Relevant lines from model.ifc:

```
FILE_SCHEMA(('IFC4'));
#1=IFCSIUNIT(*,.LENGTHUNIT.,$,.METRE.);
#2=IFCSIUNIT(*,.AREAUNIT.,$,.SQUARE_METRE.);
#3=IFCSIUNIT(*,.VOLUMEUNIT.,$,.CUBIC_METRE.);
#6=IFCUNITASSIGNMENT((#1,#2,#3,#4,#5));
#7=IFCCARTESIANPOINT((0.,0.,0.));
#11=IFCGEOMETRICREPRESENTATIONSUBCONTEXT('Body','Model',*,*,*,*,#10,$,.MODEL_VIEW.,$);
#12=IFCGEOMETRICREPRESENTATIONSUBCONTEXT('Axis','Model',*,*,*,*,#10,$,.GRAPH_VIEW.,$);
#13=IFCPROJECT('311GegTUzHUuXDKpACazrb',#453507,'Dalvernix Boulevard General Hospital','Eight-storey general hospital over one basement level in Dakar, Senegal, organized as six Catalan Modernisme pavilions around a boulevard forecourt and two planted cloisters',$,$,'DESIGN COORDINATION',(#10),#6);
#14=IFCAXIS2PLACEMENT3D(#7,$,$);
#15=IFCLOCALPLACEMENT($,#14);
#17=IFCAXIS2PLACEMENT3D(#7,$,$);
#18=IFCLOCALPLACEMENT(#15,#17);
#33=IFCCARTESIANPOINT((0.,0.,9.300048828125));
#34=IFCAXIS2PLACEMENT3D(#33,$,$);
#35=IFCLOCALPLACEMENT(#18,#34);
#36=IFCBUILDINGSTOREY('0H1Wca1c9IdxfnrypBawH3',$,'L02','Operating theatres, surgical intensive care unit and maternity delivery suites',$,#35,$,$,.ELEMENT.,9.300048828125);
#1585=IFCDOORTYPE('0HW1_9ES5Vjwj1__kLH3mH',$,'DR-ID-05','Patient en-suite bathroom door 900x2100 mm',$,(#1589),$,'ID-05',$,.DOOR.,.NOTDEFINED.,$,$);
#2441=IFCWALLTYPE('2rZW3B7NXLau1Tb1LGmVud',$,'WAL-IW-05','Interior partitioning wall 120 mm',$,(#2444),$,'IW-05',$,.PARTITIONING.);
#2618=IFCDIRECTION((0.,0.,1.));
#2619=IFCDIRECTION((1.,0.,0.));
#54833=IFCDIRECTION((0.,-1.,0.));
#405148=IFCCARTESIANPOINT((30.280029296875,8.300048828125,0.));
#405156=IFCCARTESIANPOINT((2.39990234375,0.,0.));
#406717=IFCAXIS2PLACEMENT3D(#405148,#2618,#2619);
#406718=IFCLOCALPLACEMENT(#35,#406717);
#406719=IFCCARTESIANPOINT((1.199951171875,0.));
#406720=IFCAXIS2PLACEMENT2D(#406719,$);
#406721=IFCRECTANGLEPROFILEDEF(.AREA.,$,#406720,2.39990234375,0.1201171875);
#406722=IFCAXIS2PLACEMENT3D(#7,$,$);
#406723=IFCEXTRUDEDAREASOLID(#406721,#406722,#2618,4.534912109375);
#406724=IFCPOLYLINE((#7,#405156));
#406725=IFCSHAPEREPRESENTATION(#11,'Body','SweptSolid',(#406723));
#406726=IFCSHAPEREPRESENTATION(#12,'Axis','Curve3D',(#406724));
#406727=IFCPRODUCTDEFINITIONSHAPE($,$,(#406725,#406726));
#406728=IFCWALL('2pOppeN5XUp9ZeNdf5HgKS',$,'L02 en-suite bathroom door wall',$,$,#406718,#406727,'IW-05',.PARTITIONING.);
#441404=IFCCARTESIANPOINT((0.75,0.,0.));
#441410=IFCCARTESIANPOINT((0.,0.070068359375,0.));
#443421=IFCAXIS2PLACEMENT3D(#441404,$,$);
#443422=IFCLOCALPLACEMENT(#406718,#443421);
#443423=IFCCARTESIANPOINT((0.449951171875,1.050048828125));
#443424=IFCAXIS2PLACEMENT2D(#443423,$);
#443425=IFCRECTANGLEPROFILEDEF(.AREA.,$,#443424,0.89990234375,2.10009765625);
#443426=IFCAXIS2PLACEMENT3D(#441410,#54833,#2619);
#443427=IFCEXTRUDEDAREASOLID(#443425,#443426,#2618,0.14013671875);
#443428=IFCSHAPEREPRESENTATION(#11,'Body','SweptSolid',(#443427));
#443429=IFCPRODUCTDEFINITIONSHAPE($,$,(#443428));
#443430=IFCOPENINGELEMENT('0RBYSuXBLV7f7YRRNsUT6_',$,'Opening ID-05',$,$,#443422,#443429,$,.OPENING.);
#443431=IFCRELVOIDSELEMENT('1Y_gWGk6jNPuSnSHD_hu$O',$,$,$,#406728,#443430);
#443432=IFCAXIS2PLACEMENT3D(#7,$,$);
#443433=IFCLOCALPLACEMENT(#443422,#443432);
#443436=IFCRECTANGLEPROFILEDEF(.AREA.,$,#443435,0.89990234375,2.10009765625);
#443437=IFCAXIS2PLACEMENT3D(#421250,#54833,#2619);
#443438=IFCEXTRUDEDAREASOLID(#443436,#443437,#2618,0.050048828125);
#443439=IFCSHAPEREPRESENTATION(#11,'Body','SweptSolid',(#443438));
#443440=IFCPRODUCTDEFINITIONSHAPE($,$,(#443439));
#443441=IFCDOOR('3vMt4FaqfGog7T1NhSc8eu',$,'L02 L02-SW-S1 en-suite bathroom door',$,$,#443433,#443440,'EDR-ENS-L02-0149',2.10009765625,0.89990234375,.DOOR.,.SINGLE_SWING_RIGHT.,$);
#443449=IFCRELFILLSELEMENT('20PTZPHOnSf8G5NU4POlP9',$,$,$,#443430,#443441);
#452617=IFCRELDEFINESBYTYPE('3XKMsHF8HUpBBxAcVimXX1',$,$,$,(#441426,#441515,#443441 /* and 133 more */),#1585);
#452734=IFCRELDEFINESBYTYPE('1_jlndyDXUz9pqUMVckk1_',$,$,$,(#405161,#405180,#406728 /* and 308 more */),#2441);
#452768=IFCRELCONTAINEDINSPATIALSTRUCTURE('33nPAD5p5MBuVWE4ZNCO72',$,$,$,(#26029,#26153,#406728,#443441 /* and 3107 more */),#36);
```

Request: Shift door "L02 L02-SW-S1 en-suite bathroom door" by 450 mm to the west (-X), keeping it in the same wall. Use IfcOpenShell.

```python
import ifcopenshell
import ifcopenshell.api.geometry
import ifcopenshell.util.placement

model = ifcopenshell.open("model.ifc")

door = model.by_guid("3vMt4FaqfGog7T1NhSc8eu")
opening = door.FillsVoids[0].RelatingOpeningElement
wall = opening.VoidsElements[0].RelatingBuildingElement

wall_matrix = ifcopenshell.util.placement.get_local_placement(wall.ObjectPlacement)
shift = wall_matrix[:3, 0] * -0.45
before = ifcopenshell.util.placement.get_local_placement(door.ObjectPlacement)[:3, 3].copy()

# The door is placed relative to its opening, so it follows when the opening moves.
matrix = ifcopenshell.util.placement.get_local_placement(opening.ObjectPlacement)
matrix[:3, 3] += shift
ifcopenshell.api.geometry.edit_object_placement(
    model, product=opening, matrix=matrix, is_si=False, should_transform_children=True
)

after = ifcopenshell.util.placement.get_local_placement(door.ObjectPlacement)[:3, 3]
print("door moved by", (after - before).round(3) + 0.0)

model.write("model_updated.ifc")
```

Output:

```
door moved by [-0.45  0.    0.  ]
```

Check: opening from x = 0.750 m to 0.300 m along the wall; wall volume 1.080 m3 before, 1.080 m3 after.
